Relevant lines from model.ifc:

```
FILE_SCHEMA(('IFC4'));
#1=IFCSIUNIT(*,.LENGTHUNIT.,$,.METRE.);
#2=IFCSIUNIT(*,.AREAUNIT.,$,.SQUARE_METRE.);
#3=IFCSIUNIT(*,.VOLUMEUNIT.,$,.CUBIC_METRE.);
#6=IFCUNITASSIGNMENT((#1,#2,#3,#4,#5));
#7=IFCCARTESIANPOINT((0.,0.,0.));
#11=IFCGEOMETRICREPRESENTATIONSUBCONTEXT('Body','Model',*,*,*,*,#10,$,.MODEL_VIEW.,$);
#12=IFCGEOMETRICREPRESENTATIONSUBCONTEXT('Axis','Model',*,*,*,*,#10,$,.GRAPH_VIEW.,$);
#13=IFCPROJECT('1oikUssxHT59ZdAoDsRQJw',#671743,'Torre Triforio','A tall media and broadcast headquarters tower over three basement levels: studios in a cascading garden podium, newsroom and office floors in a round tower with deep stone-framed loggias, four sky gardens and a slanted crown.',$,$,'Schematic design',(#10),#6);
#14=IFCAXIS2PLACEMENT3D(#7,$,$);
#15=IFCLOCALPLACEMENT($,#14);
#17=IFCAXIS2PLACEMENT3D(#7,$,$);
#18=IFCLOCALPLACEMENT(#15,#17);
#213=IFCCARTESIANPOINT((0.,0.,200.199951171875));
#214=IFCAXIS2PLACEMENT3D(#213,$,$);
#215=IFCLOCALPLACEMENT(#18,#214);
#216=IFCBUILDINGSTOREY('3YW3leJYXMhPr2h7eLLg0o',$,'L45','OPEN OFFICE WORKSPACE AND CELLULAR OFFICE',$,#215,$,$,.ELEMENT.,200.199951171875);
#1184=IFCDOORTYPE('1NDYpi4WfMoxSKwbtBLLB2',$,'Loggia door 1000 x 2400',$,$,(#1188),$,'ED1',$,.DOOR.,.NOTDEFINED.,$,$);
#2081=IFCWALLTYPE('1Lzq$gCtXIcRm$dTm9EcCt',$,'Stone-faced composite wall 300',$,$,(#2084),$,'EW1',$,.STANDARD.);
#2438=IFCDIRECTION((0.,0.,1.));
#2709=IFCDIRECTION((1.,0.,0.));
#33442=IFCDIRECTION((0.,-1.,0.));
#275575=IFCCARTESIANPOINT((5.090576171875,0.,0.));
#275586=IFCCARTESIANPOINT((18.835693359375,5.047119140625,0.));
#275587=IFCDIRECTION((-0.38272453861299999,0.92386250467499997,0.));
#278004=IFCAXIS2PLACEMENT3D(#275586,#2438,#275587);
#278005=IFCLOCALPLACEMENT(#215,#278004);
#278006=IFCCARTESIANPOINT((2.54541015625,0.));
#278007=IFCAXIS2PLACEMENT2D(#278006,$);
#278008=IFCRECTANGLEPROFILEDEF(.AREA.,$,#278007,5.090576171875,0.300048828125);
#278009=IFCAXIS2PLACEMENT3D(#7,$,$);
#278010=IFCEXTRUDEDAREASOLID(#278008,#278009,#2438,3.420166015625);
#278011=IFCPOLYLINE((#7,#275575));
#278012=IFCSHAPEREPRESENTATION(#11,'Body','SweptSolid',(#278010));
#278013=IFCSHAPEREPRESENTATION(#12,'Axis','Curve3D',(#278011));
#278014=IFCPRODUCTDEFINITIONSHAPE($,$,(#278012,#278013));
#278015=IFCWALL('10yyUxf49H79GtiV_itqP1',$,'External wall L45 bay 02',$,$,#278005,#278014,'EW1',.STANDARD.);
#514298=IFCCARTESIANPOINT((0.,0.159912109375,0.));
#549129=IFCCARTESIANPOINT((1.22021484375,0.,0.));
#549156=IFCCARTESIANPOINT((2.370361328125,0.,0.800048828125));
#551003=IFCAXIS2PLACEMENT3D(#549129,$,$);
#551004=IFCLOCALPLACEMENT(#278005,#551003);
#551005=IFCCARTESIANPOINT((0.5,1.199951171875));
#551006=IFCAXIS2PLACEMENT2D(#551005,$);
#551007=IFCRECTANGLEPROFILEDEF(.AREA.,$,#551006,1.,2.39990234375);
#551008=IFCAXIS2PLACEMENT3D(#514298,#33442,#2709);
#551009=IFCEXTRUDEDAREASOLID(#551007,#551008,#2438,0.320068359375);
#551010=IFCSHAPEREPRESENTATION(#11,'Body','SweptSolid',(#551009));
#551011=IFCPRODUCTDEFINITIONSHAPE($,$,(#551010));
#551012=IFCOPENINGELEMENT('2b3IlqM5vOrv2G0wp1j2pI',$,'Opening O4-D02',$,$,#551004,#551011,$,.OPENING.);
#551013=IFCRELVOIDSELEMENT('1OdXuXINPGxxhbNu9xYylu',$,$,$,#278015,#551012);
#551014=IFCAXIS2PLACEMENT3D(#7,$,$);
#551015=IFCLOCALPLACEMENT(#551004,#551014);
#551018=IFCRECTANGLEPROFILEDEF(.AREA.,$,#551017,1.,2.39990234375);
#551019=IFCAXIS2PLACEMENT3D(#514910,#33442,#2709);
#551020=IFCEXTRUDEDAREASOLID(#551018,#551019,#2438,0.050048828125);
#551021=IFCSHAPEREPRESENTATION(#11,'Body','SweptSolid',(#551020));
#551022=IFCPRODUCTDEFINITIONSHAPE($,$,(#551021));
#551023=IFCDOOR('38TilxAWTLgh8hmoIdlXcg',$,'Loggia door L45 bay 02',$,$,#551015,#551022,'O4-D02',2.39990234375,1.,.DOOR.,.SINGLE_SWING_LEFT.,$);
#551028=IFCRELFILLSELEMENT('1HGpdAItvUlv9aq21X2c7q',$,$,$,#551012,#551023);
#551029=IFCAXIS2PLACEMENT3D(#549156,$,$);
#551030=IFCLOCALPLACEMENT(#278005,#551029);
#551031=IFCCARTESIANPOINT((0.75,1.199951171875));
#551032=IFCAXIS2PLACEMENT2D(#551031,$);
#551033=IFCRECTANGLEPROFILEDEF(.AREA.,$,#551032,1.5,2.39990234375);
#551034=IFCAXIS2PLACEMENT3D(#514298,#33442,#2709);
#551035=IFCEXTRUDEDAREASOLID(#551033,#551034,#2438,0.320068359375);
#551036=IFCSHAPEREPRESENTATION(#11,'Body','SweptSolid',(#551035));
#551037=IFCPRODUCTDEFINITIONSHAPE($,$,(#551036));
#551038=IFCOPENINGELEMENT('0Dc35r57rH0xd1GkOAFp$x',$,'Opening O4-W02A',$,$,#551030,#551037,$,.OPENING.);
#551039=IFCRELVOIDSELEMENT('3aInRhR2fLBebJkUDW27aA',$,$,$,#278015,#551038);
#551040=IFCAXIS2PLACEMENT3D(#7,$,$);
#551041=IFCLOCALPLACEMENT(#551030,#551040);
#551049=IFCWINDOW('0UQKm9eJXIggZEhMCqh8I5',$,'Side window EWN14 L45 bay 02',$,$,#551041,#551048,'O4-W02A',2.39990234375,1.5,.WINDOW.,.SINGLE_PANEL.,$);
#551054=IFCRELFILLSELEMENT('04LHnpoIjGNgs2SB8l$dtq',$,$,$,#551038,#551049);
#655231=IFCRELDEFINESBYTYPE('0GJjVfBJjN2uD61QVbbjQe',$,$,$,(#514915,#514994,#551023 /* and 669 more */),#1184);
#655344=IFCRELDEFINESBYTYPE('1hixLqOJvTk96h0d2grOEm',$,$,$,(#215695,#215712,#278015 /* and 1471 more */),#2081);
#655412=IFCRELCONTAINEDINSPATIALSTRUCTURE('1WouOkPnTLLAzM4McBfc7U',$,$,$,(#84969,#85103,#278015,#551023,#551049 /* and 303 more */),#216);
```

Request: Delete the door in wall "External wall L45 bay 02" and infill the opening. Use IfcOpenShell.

```python
import ifcopenshell
import ifcopenshell.api.feature
import ifcopenshell.api.root
import ifcopenshell.geom
import ifcopenshell.util.shape

model = ifcopenshell.open("model.ifc")
settings = ifcopenshell.geom.settings()


def volume(element):
    """Net volume in cubic metres, openings subtracted."""
    shape = ifcopenshell.geom.create_shape(settings, element)
    return ifcopenshell.util.shape.get_volume(shape.geometry)


door = model.by_guid("38TilxAWTLgh8hmoIdlXcg")
opening = door.FillsVoids[0].RelatingOpeningElement
wall = opening.VoidsElements[0].RelatingBuildingElement
before = volume(wall)

ifcopenshell.api.root.remove_product(model, product=door)
ifcopenshell.api.feature.remove_feature(model, feature=opening)

after = volume(wall)

print(f"wall volume {before:.3f} -> {after:.3f} m3")

model.write("model_edited.ifc")
```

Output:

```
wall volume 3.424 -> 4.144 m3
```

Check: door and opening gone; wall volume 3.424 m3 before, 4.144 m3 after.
